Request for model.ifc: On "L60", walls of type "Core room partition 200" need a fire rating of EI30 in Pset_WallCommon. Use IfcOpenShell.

First a look at what the model holds.

```python
import ifcopenshell
import ifcopenshell.util.element

model = ifcopenshell.open("model.ifc")
print(model.schema)
storey = next(s for s in model.by_type("IfcBuildingStorey") if s.Name == "L60")
walls = [e for e in ifcopenshell.util.element.get_decomposition(storey) if e.is_a("IfcWall")]
seen = {}
for e in walls:
    element_type = ifcopenshell.util.element.get_type(e)
    key = (element_type.Name if element_type != e and element_type else None, ifcopenshell.util.element.get_pset(e, "Pset_WallCommon", "FireRating"))
    seen[key] = seen.get(key, 0) + 1
for (name, value), count in sorted(seen.items(), key=str):
    print(count, "x", name, "|", value)
```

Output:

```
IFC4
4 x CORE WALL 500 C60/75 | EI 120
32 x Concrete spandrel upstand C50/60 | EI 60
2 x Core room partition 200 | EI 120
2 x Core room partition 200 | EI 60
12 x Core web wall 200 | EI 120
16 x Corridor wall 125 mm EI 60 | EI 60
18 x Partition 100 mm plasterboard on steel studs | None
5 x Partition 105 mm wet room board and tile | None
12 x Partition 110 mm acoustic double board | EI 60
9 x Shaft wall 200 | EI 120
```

```python
import ifcopenshell
import ifcopenshell.api.pset
import ifcopenshell.util.element

model = ifcopenshell.open("model.ifc")

storey = next(s for s in model.by_type("IfcBuildingStorey") if s.Name == "L60")
walls = [e for e in ifcopenshell.util.element.get_decomposition(storey) if e.is_a("IfcWall")]

count = 0
for e in walls:
    element_type = ifcopenshell.util.element.get_type(e)
    if element_type in (None, e) or element_type.Name != "Core room partition 200":
        continue
    # add_pset returns the element's existing set when there is one.
    pset = ifcopenshell.api.pset.add_pset(model, product=e, name="Pset_WallCommon")
    ifcopenshell.api.pset.edit_pset(model, pset=pset, properties={"FireRating": "EI30"})
    count += 1

print(count, "walls updated")

model.write("model_updated.ifc")
```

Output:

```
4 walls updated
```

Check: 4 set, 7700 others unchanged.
